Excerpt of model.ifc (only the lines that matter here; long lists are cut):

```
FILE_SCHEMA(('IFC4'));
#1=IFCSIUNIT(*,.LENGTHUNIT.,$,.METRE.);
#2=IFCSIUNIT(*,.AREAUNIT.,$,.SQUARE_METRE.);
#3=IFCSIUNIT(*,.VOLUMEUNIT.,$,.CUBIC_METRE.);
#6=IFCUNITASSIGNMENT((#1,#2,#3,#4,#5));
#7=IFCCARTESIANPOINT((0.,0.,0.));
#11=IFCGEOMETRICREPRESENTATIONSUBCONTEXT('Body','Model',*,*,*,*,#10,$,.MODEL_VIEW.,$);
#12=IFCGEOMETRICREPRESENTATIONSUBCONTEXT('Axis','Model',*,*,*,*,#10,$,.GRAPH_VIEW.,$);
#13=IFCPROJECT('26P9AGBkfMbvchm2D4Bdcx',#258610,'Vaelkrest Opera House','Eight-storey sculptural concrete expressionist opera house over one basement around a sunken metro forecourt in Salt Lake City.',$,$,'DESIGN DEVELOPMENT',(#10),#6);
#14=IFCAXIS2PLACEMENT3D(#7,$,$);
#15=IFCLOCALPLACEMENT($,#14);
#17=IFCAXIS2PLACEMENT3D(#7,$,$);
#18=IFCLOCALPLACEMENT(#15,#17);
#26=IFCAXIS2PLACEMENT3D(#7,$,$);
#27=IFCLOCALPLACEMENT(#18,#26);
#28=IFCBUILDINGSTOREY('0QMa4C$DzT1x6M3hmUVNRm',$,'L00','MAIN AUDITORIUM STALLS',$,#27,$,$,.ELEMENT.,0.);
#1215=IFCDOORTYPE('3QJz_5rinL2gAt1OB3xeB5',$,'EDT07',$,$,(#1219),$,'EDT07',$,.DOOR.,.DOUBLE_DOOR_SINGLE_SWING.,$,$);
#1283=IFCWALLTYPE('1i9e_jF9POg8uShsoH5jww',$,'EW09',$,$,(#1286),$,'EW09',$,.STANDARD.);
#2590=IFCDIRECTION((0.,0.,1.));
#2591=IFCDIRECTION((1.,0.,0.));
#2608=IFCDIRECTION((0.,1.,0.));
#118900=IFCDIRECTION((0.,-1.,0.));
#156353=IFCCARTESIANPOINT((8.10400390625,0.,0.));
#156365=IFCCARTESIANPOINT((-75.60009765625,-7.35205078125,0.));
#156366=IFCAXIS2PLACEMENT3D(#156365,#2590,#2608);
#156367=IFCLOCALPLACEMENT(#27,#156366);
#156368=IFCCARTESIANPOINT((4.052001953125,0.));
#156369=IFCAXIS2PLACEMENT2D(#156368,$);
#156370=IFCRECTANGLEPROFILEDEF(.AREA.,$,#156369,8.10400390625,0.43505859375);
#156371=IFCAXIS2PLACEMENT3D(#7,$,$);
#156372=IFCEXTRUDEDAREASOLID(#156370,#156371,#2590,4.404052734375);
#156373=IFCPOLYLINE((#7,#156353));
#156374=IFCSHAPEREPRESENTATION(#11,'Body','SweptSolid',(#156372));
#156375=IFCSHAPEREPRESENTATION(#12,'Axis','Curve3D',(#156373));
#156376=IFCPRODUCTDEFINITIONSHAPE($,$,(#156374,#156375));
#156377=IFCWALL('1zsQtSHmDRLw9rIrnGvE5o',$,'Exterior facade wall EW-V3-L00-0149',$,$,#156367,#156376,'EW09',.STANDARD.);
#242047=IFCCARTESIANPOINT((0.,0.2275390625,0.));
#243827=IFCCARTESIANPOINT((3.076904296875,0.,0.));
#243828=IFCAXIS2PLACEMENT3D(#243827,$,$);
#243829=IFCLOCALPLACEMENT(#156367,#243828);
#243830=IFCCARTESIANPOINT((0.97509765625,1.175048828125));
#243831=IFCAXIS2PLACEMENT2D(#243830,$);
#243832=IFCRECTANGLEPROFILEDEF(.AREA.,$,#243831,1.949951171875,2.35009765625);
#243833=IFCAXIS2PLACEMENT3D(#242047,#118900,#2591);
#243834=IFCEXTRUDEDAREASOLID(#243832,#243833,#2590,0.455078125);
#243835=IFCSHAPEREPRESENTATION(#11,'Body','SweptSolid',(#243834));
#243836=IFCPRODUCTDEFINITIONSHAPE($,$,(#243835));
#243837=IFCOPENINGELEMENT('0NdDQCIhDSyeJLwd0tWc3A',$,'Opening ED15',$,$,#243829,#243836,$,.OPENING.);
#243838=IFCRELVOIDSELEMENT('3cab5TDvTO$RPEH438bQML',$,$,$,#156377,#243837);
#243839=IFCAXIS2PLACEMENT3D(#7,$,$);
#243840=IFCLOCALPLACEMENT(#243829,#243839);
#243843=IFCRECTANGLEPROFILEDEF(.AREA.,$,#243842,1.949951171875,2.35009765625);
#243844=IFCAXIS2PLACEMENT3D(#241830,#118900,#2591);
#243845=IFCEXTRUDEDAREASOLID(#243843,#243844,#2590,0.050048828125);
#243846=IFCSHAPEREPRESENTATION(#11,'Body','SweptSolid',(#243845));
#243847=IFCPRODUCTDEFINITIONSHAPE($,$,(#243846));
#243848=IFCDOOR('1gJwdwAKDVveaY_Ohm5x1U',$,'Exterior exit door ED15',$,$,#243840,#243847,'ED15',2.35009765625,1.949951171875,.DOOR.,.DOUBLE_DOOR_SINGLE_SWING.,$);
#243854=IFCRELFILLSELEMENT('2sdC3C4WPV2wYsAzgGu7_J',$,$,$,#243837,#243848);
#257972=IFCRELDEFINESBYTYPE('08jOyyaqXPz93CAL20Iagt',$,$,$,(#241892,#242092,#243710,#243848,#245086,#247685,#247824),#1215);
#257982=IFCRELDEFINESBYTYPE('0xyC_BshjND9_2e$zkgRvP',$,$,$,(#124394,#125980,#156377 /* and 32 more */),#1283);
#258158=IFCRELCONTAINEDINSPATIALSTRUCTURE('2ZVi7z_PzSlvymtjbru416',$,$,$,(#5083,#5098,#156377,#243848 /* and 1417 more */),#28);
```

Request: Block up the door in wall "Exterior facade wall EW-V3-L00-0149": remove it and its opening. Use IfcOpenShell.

```python
import ifcopenshell
import ifcopenshell.api.feature
import ifcopenshell.api.root
import ifcopenshell.geom
import ifcopenshell.util.shape

model = ifcopenshell.open("model.ifc")
settings = ifcopenshell.geom.settings()


def volume(element):
    """Net volume in cubic metres, openings subtracted."""
    shape = ifcopenshell.geom.create_shape(settings, element)
    return ifcopenshell.util.shape.get_volume(shape.geometry)


door = model.by_guid("1gJwdwAKDVveaY_Ohm5x1U")
opening = door.FillsVoids[0].RelatingOpeningElement
wall = opening.VoidsElements[0].RelatingBuildingElement
before = volume(wall)

ifcopenshell.api.root.remove_product(model, product=door)
ifcopenshell.api.feature.remove_feature(model, feature=opening)

after = volume(wall)

print(f"wall volume {before:.3f} -> {after:.3f} m3")

model.write("model_updated.ifc")
```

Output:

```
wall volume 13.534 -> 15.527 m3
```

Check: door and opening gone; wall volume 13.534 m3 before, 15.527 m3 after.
